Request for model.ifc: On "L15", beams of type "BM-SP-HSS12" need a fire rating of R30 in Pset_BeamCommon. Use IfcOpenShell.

First a look at what the model holds.

```python
import ifcopenshell
import ifcopenshell.util.element

model = ifcopenshell.open("model.ifc")
print(model.schema)
storey = next(s for s in model.by_type("IfcBuildingStorey") if s.Name == "L15")
beams = [e for e in ifcopenshell.util.element.get_decomposition(storey) if e.is_a("IfcBeam")]
seen = {}
for e in beams:
    element_type = ifcopenshell.util.element.get_type(e)
    key = (element_type.Name if element_type != e and element_type else None, ifcopenshell.util.element.get_pset(e, "Pset_BeamCommon", "FireRating"))
    seen[key] = seen.get(key, 0) + 1
for (name, value), count in sorted(seen.items(), key=str):
    print(count, "x", name, "|", value)
```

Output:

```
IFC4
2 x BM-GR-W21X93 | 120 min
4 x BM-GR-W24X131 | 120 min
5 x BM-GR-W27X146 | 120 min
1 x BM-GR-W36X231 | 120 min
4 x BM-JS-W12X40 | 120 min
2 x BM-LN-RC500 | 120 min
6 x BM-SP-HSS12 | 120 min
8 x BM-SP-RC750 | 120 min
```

```python
import ifcopenshell
import ifcopenshell.api.pset
import ifcopenshell.util.element

model = ifcopenshell.open("model.ifc")

storey = next(s for s in model.by_type("IfcBuildingStorey") if s.Name == "L15")
beams = [e for e in ifcopenshell.util.element.get_decomposition(storey) if e.is_a("IfcBeam")]

count = 0
for e in beams:
    element_type = ifcopenshell.util.element.get_type(e)
    if element_type in (None, e) or element_type.Name != "BM-SP-HSS12":
        continue
    # add_pset returns the element's existing set when there is one.
    pset = ifcopenshell.api.pset.add_pset(model, product=e, name="Pset_BeamCommon")
    ifcopenshell.api.pset.edit_pset(model, pset=pset, properties={"FireRating": "R30"})
    count += 1

print(count, "beams updated")

model.write("model-out.ifc")
```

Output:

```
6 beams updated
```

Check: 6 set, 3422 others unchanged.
